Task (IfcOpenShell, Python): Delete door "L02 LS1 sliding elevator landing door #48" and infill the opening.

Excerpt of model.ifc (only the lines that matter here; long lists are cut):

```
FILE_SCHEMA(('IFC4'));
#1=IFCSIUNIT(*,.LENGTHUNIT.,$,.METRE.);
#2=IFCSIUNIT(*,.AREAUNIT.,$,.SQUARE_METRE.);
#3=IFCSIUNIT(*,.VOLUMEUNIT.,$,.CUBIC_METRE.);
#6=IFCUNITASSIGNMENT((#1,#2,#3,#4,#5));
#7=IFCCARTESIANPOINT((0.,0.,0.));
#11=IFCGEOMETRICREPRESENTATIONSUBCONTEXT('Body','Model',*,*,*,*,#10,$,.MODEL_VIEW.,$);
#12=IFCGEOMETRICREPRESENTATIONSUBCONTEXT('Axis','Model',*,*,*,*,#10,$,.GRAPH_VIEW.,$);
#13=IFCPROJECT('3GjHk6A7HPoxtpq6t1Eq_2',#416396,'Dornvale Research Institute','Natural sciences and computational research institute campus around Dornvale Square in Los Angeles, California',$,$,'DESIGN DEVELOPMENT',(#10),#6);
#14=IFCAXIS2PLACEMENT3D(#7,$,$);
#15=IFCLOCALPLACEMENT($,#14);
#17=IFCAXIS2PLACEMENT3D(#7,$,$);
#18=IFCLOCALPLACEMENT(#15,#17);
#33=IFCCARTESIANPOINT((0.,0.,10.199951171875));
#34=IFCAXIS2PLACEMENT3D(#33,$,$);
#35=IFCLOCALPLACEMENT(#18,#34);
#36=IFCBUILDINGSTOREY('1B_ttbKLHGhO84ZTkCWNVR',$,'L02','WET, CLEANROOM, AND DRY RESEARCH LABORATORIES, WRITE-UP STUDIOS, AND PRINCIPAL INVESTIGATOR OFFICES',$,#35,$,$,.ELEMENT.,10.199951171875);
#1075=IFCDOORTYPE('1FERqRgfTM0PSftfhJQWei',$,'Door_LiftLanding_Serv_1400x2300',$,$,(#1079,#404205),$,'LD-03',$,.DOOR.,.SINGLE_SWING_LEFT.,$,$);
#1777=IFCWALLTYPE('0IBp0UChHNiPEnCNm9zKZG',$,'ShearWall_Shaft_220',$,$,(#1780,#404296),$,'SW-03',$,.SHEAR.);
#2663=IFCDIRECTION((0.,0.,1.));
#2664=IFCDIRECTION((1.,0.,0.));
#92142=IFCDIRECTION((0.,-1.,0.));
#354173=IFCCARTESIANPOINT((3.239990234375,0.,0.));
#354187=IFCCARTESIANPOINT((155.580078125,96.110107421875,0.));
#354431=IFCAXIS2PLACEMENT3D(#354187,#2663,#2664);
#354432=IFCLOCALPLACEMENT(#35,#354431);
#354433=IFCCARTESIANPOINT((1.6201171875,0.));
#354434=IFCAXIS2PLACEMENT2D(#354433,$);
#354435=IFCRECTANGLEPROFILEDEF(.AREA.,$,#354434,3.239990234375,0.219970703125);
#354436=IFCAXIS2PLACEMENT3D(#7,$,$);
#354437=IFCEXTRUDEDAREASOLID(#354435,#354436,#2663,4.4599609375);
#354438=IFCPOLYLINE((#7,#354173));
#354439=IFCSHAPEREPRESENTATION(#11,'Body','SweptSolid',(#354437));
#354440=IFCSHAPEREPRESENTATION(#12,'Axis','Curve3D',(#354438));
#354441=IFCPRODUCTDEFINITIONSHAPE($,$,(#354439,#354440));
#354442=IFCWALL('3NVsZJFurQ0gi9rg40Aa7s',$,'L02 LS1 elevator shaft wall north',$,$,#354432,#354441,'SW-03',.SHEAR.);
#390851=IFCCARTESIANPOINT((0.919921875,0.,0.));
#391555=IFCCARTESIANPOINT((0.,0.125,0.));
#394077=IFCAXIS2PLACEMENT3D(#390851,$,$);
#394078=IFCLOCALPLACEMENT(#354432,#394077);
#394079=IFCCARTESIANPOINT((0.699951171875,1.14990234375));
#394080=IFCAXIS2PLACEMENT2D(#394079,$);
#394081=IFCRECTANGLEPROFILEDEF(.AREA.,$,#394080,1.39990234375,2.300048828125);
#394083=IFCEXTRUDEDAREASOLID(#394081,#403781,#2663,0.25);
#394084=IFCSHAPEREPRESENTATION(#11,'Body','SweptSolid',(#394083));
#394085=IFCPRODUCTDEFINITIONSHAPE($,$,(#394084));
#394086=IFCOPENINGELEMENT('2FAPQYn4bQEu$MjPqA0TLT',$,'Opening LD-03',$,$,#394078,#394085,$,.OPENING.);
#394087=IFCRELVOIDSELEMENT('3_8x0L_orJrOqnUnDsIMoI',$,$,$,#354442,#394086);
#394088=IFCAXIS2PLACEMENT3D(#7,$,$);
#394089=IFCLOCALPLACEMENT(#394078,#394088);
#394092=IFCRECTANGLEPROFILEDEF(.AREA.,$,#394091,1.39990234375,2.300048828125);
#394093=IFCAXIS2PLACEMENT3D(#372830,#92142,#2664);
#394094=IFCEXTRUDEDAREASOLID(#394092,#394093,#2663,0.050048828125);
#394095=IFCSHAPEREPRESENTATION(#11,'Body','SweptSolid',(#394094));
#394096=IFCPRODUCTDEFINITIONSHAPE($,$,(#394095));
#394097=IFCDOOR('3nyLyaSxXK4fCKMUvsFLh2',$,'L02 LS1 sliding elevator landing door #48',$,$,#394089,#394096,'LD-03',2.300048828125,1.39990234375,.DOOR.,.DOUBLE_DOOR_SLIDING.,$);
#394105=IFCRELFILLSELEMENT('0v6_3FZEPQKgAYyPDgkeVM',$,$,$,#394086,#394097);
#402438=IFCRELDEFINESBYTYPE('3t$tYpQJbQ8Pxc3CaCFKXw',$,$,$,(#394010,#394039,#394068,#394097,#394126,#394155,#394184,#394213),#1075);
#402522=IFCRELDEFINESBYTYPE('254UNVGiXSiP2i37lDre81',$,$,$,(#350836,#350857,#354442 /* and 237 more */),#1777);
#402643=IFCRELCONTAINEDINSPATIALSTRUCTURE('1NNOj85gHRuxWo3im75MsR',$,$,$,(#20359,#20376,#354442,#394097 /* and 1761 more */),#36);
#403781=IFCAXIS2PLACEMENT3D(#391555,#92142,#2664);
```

```python
import ifcopenshell
import ifcopenshell.api.feature
import ifcopenshell.api.root
import ifcopenshell.geom
import ifcopenshell.util.shape

model = ifcopenshell.open("model.ifc")
settings = ifcopenshell.geom.settings()


def volume(element):
    """Net volume in cubic metres, openings subtracted."""
    shape = ifcopenshell.geom.create_shape(settings, element)
    return ifcopenshell.util.shape.get_volume(shape.geometry)


door = model.by_guid("3nyLyaSxXK4fCKMUvsFLh2")
opening = door.FillsVoids[0].RelatingOpeningElement
wall = opening.VoidsElements[0].RelatingBuildingElement
before = volume(wall)

ifcopenshell.api.root.remove_product(model, product=door)
ifcopenshell.api.feature.remove_feature(model, feature=opening)

after = volume(wall)

print(f"wall volume {before:.3f} -> {after:.3f} m3")

model.write("model_v2.ifc")
```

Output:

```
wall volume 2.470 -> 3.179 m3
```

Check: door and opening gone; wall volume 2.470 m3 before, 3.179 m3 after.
